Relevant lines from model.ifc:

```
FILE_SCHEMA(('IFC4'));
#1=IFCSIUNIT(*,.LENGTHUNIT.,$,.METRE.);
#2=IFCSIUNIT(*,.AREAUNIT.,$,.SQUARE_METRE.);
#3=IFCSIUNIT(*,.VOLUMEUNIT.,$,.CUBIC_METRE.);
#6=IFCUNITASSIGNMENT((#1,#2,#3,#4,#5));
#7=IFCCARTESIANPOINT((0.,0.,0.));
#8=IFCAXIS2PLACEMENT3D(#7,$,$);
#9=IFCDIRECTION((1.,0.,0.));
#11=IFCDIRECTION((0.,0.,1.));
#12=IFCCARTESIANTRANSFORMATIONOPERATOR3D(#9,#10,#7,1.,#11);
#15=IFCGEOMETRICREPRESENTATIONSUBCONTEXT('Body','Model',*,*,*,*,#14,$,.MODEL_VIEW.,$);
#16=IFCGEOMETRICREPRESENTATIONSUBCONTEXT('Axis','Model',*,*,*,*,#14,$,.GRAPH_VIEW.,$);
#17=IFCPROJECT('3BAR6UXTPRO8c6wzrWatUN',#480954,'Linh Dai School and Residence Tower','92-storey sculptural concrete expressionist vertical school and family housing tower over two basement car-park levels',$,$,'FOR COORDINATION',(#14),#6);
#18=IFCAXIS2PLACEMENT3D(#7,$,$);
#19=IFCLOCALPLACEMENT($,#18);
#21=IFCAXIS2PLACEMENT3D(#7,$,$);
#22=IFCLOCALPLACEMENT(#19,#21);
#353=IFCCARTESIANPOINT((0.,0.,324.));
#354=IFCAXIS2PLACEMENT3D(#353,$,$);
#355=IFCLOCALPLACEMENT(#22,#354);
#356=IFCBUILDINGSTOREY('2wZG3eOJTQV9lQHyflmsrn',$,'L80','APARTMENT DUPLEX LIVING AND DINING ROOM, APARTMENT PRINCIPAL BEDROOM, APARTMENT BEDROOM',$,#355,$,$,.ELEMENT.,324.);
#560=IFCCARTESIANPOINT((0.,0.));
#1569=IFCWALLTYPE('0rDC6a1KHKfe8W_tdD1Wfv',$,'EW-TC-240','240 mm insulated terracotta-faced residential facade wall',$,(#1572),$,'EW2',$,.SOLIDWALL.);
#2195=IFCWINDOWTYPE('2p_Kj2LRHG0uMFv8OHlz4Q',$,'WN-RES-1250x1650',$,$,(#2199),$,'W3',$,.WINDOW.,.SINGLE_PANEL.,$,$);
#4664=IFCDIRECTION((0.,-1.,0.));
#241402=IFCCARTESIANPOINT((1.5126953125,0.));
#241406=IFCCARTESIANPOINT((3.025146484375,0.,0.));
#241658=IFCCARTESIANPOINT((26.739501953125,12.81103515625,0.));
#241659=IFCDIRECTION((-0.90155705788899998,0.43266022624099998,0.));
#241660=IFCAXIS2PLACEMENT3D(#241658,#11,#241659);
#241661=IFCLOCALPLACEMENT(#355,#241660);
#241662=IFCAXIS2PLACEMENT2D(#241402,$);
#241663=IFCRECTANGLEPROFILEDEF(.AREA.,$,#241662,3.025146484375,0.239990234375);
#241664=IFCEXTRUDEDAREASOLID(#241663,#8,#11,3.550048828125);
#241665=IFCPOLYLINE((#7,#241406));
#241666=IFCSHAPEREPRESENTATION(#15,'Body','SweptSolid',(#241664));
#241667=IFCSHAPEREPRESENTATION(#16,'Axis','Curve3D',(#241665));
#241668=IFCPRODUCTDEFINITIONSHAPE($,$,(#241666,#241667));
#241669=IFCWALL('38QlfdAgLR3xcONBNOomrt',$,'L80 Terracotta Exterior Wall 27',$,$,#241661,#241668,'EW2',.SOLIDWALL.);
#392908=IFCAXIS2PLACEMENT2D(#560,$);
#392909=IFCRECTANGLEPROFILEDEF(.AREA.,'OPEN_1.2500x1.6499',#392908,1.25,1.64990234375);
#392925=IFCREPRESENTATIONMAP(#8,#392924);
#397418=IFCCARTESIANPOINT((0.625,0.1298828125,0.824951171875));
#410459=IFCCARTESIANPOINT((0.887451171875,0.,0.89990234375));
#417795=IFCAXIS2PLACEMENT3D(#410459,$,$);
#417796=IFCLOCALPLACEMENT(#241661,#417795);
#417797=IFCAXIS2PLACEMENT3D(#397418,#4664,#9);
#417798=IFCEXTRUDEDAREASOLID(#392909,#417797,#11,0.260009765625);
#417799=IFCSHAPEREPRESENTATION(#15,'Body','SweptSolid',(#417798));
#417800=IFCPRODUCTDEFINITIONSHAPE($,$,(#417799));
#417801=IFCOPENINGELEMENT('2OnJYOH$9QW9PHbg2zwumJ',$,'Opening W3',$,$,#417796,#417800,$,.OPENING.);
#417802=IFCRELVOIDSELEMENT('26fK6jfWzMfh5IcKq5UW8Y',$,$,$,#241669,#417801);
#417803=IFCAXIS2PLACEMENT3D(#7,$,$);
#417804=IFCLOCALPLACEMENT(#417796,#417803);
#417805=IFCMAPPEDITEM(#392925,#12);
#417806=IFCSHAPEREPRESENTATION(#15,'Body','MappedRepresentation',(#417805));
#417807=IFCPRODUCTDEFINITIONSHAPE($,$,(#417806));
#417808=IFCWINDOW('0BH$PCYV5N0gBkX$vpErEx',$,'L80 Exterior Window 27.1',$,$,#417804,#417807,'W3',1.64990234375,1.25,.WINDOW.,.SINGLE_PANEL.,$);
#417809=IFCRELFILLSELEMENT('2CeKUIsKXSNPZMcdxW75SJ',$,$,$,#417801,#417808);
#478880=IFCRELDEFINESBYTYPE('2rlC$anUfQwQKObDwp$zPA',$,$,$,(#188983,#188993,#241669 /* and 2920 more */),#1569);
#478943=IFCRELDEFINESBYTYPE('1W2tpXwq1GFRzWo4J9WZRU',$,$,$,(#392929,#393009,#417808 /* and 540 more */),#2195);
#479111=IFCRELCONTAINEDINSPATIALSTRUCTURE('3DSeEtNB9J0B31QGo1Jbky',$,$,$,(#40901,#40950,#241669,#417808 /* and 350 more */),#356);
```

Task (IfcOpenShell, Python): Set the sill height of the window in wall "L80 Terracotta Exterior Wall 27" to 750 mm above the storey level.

```python
import numpy as np
import ifcopenshell
import ifcopenshell.api.geometry
import ifcopenshell.geom
import ifcopenshell.util.element
import ifcopenshell.util.placement
import ifcopenshell.util.shape
import ifcopenshell.util.unit

model = ifcopenshell.open("model.ifc")
unit_scale = ifcopenshell.util.unit.calculate_unit_scale(model)

window = model.by_guid("0BH$PCYV5N0gBkX$vpErEx")
opening = window.FillsVoids[0].RelatingOpeningElement
storey = ifcopenshell.util.element.get_container(window, ifc_class="IfcBuildingStorey")
level = ifcopenshell.util.placement.get_local_placement(storey.ObjectPlacement)[2, 3]

# The opening's origin need not be at the sill, so measure its lowest point.
shape = ifcopenshell.geom.create_shape(ifcopenshell.geom.settings(), opening)
bottom = ifcopenshell.util.shape.get_shape_bottom_elevation(shape, shape.geometry) / unit_scale
dz = level + 0.75 - bottom

shift = np.array([0.0, 0.0, dz])
# The window is placed relative to its opening, so it follows when the opening moves.
matrix = ifcopenshell.util.placement.get_local_placement(opening.ObjectPlacement)
matrix[:3, 3] += shift
ifcopenshell.api.geometry.edit_object_placement(
    model, product=opening, matrix=matrix, is_si=False, should_transform_children=True
)

print(f"moved by {dz * unit_scale:+.3f} m")

model.write("model-out.ifc")
```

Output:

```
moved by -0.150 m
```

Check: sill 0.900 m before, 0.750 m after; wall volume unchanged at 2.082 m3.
